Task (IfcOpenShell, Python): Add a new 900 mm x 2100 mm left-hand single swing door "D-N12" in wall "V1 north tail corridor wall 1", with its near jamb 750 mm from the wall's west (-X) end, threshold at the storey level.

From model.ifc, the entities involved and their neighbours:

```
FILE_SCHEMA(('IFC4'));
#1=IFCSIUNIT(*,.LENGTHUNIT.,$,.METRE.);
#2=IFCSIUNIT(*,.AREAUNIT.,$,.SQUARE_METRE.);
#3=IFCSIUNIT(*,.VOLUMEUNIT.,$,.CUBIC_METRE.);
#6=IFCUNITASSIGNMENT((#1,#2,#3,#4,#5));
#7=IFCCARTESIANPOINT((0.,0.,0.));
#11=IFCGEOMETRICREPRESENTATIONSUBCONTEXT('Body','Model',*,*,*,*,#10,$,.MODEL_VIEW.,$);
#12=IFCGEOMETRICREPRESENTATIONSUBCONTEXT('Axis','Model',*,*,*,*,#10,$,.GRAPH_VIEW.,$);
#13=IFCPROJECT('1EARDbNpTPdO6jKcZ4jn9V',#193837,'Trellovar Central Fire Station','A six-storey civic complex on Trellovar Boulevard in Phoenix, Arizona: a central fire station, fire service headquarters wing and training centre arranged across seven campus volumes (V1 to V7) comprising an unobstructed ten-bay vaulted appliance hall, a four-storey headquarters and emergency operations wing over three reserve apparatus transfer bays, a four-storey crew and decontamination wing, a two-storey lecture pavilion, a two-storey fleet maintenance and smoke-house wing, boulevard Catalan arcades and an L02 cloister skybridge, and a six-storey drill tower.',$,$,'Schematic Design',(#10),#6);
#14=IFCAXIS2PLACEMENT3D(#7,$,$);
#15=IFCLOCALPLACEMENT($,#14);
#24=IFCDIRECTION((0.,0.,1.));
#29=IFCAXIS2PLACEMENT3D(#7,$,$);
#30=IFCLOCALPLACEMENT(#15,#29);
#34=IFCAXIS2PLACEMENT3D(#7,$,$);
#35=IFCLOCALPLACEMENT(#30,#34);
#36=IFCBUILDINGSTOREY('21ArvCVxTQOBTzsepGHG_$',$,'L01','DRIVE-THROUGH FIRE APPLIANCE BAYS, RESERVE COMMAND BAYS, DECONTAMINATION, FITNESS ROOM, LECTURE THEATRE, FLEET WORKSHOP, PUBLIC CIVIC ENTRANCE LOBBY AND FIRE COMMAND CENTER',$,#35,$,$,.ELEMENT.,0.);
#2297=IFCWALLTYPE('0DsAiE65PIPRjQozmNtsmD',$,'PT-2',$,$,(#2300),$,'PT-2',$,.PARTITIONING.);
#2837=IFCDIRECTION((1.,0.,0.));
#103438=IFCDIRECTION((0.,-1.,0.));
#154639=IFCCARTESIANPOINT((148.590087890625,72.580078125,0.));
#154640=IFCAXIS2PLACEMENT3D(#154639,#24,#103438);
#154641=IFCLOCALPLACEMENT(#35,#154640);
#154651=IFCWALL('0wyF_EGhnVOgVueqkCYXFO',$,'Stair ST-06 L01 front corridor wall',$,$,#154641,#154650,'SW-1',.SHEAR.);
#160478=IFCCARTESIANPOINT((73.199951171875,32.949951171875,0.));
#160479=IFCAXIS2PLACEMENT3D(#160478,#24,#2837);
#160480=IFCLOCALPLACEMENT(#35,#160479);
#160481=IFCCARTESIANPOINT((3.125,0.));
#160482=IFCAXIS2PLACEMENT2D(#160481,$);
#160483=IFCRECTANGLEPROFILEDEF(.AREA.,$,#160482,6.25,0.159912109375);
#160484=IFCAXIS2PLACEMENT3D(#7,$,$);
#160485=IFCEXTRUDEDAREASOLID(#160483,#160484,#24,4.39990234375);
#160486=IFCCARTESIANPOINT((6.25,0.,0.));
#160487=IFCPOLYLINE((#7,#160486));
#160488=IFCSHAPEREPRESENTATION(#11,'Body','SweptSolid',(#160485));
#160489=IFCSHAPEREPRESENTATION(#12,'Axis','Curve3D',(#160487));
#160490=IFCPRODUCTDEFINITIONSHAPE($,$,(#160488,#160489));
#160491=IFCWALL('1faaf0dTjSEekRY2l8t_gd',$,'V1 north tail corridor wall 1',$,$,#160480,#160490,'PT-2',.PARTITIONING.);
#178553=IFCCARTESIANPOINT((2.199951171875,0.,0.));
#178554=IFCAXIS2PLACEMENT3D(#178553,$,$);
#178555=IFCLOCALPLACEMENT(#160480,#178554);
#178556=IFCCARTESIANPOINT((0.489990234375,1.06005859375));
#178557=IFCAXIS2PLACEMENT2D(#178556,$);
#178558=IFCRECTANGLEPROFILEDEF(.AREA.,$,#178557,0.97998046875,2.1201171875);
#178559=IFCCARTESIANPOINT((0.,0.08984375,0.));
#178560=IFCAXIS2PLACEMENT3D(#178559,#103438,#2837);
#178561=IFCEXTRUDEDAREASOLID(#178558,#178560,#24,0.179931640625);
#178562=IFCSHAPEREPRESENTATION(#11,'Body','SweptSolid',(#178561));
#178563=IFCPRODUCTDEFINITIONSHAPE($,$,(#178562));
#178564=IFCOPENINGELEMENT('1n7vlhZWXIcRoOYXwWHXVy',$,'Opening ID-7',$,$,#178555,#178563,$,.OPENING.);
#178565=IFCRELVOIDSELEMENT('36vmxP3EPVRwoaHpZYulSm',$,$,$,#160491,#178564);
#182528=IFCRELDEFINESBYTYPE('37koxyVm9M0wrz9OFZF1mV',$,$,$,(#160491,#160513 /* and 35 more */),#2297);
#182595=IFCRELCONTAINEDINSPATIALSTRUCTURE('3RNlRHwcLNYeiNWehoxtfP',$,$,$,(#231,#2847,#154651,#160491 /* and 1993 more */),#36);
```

```python
import numpy as np
import ifcopenshell
import ifcopenshell.api.feature
import ifcopenshell.api.geometry
import ifcopenshell.api.root
import ifcopenshell.api.spatial
import ifcopenshell.geom
import ifcopenshell.util.element
import ifcopenshell.util.placement
import ifcopenshell.util.representation
import ifcopenshell.util.shape
import ifcopenshell.util.unit

model = ifcopenshell.open("model.ifc")
unit_scale = ifcopenshell.util.unit.calculate_unit_scale(model)
settings = ifcopenshell.geom.settings()


def volume(element):
    """Net volume in cubic metres, openings subtracted."""
    shape = ifcopenshell.geom.create_shape(settings, element)
    return ifcopenshell.util.shape.get_volume(shape.geometry)


wall = model.by_guid("1faaf0dTjSEekRY2l8t_gd")
storey = ifcopenshell.util.element.get_container(wall, ifc_class="IfcBuildingStorey")
context = ifcopenshell.util.representation.get_context(model, "Model", "Body", "MODEL_VIEW")
before = volume(wall)

width, height, from_end, sill = 0.9, 2.1, 0.75, 0.0  # metres

# The wall runs along its own X axis, and the end named is its -X end.
wall_shape = ifcopenshell.geom.create_shape(settings, wall)
x, y, z = ifcopenshell.util.shape.get_vertices(wall_shape.geometry).T
start = x.min() + from_end
face, thickness = float(y.min()), float(y.max() - y.min())
wall_matrix = ifcopenshell.util.placement.get_local_placement(wall.ObjectPlacement)
level = ifcopenshell.util.placement.get_local_placement(storey.ObjectPlacement)[2, 3]


def in_wall(x, y):
    """Placement at x, y metres in the wall's axes, at sill height."""
    matrix = wall_matrix.copy()
    matrix[:, 3] = wall_matrix @ np.array([x / unit_scale, y / unit_scale, 0.0, 1.0])
    matrix[2, 3] = level + sill / unit_scale
    return matrix


# Opening: a box that overshoots both wall faces by 50 mm.
opening = ifcopenshell.api.root.create_entity(model, ifc_class="IfcOpeningElement", predefined_type="OPENING")
box = ifcopenshell.api.geometry.add_wall_representation(
    model, context=context, length=width, height=height, thickness=thickness + 0.1
)
ifcopenshell.api.geometry.assign_representation(model, product=opening, representation=box)
ifcopenshell.api.geometry.edit_object_placement(model, product=opening, matrix=in_wall(start, face - 0.05), is_si=False)
ifcopenshell.api.feature.add_feature(model, feature=opening, element=wall)

door = ifcopenshell.api.root.create_entity(model, ifc_class="IfcDoor", name="D-N12", predefined_type="DOOR")
door.OverallWidth, door.OverallHeight = width / unit_scale, height / unit_scale
door.OperationType = "SINGLE_SWING_LEFT"
body = ifcopenshell.api.geometry.add_door_representation(
    model,
    context=context,
    overall_width=door.OverallWidth,
    overall_height=door.OverallHeight,
    operation_type="SINGLE_SWING_LEFT",
    lining_properties={"LiningDepth": thickness / unit_scale, "ThresholdDepth": thickness / unit_scale},
)
ifcopenshell.api.geometry.assign_representation(model, product=door, representation=body)
ifcopenshell.api.spatial.assign_container(model, products=[door], relating_structure=storey)
ifcopenshell.api.feature.add_filling(model, opening=opening, element=door)

# The lining spans the wall, so the door starts at the wall face.
ifcopenshell.api.geometry.edit_object_placement(model, product=door, matrix=in_wall(start, face), is_si=False)

after = volume(wall)

print(f"wall volume {before:.3f} -> {after:.3f} m3")

model.write("model_updated.ifc")
```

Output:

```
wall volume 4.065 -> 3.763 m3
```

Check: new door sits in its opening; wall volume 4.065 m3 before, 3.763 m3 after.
